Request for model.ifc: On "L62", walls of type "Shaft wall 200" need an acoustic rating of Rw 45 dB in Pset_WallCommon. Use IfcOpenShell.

First a look at what the model holds.

```python
import ifcopenshell
import ifcopenshell.util.element

model = ifcopenshell.open("model.ifc")
print(model.schema)
storey = next(s for s in model.by_type("IfcBuildingStorey") if s.Name == "L62")
walls = [e for e in ifcopenshell.util.element.get_decomposition(storey) if e.is_a("IfcWall")]
seen = {}
for e in walls:
    element_type = ifcopenshell.util.element.get_type(e)
    key = (element_type.Name if element_type != e and element_type else None, ifcopenshell.util.element.get_pset(e, "Pset_WallCommon", "AcousticRating"))
    seen[key] = seen.get(key, 0) + 1
for (name, value), count in sorted(seen.items(), key=str):
    print(count, "x", name, "|", value)
```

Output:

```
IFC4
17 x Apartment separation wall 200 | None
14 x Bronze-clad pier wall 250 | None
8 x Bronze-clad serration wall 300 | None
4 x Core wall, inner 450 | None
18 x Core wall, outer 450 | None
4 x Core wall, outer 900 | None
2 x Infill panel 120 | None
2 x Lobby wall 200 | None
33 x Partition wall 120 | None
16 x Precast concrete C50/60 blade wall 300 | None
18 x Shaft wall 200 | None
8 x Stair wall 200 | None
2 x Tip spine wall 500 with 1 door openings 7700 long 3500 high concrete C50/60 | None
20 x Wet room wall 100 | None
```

```python
import ifcopenshell
import ifcopenshell.api.pset
import ifcopenshell.util.element

model = ifcopenshell.open("model.ifc")

storey = next(s for s in model.by_type("IfcBuildingStorey") if s.Name == "L62")
walls = [e for e in ifcopenshell.util.element.get_decomposition(storey) if e.is_a("IfcWall")]

count = 0
for e in walls:
    element_type = ifcopenshell.util.element.get_type(e)
    if element_type in (None, e) or element_type.Name != "Shaft wall 200":
        continue
    found = ifcopenshell.util.element.get_pset(e, "Pset_WallCommon", should_inherit=False)
    if found:
        pset = model.by_id(found["id"])
        if len(ifcopenshell.util.element.get_elements_by_pset(pset)) > 1:
            pset = ifcopenshell.api.pset.unshare_pset(model, products=[e], pset=pset)[0]
    else:
        pset = ifcopenshell.api.pset.add_pset(model, product=e, name="Pset_WallCommon")
    ifcopenshell.api.pset.edit_pset(model, pset=pset, properties={"AcousticRating": "Rw 45 dB"})
    count += 1

print(count, "walls updated")

model.write("model_edited.ifc")
```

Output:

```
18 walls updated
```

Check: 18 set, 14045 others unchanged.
